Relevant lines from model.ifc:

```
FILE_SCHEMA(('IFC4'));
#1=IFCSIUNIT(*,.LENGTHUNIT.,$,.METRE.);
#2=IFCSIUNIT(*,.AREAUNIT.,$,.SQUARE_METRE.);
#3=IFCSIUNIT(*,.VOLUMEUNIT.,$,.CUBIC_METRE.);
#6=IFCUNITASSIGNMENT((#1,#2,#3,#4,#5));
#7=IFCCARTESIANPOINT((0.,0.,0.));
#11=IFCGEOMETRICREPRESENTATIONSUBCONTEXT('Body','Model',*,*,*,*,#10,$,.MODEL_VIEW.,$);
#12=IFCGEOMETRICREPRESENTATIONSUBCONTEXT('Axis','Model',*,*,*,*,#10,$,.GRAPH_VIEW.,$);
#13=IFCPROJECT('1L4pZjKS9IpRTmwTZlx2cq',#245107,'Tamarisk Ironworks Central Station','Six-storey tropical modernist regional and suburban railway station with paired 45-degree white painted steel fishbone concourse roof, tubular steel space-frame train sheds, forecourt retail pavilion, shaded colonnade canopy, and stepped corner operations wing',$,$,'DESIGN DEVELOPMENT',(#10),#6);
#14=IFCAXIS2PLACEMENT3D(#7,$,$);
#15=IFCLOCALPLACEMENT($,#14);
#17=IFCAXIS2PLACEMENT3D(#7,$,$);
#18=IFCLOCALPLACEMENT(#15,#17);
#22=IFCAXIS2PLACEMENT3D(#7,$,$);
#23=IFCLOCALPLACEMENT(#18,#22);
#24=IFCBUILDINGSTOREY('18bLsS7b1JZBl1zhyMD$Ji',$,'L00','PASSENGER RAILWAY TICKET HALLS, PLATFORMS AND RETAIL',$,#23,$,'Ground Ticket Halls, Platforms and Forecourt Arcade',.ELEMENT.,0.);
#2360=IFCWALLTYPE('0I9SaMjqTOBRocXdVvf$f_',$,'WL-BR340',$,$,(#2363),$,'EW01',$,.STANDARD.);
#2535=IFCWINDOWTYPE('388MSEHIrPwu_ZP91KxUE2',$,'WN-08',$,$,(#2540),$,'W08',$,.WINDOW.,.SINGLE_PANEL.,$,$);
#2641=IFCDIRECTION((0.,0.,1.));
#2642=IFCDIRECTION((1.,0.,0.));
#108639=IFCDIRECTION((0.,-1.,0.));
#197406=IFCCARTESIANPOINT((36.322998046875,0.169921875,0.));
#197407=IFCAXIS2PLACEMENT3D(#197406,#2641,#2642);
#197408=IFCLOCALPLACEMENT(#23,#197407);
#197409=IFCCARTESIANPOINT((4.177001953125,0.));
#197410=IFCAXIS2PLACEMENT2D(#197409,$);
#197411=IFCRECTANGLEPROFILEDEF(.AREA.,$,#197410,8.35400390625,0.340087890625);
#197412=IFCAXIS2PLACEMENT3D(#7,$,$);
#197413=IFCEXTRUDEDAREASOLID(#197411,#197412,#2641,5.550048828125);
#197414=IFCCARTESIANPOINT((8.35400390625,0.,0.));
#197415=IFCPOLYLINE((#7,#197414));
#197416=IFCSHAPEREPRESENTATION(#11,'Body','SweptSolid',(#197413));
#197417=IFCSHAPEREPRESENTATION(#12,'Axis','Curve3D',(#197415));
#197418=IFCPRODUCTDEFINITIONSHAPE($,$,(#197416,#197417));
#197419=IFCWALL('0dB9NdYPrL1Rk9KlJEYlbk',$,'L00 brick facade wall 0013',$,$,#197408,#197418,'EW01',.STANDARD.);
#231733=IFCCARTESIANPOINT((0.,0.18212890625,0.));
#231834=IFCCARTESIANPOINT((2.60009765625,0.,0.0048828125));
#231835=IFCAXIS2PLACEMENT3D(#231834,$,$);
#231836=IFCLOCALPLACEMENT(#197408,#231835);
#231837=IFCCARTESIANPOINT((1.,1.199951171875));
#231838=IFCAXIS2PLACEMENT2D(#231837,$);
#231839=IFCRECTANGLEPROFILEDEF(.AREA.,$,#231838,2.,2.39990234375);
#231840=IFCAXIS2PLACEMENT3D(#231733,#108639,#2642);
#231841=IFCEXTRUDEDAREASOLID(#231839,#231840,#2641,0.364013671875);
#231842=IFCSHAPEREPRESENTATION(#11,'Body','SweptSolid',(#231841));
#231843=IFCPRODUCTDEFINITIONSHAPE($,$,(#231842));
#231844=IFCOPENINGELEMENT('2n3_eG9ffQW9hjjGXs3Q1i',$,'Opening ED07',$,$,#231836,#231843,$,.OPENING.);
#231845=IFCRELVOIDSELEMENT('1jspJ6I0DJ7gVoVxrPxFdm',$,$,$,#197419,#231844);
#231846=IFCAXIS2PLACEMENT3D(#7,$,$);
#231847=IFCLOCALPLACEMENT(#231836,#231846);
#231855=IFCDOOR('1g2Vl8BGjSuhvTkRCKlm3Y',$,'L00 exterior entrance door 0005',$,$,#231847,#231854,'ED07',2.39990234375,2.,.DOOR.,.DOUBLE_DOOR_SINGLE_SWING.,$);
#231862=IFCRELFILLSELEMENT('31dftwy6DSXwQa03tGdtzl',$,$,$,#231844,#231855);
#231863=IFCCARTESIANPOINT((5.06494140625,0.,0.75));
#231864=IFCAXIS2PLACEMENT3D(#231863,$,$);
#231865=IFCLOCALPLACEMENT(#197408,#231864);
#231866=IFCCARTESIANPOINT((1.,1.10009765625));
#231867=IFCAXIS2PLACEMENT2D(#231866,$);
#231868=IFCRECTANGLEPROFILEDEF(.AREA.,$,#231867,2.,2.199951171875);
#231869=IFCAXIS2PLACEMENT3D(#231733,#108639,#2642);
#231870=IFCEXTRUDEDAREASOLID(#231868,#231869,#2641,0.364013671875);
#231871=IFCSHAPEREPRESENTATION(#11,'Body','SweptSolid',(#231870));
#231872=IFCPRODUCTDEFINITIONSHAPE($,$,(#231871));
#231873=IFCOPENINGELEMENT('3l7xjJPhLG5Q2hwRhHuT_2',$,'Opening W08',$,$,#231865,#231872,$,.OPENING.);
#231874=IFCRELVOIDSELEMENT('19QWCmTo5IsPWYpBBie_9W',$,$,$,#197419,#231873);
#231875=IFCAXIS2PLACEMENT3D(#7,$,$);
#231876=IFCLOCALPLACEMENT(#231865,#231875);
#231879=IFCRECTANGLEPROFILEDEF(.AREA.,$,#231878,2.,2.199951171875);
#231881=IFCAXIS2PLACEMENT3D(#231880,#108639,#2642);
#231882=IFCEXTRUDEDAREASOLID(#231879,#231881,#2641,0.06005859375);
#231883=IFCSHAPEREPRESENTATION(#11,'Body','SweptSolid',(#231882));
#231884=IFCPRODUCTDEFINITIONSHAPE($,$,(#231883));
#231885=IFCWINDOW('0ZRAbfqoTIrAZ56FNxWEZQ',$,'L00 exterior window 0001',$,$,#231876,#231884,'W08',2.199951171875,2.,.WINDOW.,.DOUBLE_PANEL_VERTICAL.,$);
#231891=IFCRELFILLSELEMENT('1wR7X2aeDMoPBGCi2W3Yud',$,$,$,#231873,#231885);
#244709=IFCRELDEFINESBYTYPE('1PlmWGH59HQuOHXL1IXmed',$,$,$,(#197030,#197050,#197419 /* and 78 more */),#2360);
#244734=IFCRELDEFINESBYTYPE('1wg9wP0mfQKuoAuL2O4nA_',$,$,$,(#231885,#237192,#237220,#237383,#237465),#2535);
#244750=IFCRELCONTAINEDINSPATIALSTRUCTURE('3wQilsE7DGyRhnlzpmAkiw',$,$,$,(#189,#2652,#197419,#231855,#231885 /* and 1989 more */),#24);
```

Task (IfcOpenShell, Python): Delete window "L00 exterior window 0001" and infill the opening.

```python
import ifcopenshell
import ifcopenshell.api.feature
import ifcopenshell.api.root
import ifcopenshell.geom
import ifcopenshell.util.shape

model = ifcopenshell.open("model.ifc")
settings = ifcopenshell.geom.settings()


def volume(element):
    """Net volume in cubic metres, openings subtracted."""
    shape = ifcopenshell.geom.create_shape(settings, element)
    return ifcopenshell.util.shape.get_volume(shape.geometry)


window = model.by_guid("0ZRAbfqoTIrAZ56FNxWEZQ")
opening = window.FillsVoids[0].RelatingOpeningElement
wall = opening.VoidsElements[0].RelatingBuildingElement
before = volume(wall)

ifcopenshell.api.root.remove_product(model, product=window)
ifcopenshell.api.feature.remove_feature(model, feature=opening)

after = volume(wall)

print(f"wall volume {before:.3f} -> {after:.3f} m3")

model.write("model_v2.ifc")
```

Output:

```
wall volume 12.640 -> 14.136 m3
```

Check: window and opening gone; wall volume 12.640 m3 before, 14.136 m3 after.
